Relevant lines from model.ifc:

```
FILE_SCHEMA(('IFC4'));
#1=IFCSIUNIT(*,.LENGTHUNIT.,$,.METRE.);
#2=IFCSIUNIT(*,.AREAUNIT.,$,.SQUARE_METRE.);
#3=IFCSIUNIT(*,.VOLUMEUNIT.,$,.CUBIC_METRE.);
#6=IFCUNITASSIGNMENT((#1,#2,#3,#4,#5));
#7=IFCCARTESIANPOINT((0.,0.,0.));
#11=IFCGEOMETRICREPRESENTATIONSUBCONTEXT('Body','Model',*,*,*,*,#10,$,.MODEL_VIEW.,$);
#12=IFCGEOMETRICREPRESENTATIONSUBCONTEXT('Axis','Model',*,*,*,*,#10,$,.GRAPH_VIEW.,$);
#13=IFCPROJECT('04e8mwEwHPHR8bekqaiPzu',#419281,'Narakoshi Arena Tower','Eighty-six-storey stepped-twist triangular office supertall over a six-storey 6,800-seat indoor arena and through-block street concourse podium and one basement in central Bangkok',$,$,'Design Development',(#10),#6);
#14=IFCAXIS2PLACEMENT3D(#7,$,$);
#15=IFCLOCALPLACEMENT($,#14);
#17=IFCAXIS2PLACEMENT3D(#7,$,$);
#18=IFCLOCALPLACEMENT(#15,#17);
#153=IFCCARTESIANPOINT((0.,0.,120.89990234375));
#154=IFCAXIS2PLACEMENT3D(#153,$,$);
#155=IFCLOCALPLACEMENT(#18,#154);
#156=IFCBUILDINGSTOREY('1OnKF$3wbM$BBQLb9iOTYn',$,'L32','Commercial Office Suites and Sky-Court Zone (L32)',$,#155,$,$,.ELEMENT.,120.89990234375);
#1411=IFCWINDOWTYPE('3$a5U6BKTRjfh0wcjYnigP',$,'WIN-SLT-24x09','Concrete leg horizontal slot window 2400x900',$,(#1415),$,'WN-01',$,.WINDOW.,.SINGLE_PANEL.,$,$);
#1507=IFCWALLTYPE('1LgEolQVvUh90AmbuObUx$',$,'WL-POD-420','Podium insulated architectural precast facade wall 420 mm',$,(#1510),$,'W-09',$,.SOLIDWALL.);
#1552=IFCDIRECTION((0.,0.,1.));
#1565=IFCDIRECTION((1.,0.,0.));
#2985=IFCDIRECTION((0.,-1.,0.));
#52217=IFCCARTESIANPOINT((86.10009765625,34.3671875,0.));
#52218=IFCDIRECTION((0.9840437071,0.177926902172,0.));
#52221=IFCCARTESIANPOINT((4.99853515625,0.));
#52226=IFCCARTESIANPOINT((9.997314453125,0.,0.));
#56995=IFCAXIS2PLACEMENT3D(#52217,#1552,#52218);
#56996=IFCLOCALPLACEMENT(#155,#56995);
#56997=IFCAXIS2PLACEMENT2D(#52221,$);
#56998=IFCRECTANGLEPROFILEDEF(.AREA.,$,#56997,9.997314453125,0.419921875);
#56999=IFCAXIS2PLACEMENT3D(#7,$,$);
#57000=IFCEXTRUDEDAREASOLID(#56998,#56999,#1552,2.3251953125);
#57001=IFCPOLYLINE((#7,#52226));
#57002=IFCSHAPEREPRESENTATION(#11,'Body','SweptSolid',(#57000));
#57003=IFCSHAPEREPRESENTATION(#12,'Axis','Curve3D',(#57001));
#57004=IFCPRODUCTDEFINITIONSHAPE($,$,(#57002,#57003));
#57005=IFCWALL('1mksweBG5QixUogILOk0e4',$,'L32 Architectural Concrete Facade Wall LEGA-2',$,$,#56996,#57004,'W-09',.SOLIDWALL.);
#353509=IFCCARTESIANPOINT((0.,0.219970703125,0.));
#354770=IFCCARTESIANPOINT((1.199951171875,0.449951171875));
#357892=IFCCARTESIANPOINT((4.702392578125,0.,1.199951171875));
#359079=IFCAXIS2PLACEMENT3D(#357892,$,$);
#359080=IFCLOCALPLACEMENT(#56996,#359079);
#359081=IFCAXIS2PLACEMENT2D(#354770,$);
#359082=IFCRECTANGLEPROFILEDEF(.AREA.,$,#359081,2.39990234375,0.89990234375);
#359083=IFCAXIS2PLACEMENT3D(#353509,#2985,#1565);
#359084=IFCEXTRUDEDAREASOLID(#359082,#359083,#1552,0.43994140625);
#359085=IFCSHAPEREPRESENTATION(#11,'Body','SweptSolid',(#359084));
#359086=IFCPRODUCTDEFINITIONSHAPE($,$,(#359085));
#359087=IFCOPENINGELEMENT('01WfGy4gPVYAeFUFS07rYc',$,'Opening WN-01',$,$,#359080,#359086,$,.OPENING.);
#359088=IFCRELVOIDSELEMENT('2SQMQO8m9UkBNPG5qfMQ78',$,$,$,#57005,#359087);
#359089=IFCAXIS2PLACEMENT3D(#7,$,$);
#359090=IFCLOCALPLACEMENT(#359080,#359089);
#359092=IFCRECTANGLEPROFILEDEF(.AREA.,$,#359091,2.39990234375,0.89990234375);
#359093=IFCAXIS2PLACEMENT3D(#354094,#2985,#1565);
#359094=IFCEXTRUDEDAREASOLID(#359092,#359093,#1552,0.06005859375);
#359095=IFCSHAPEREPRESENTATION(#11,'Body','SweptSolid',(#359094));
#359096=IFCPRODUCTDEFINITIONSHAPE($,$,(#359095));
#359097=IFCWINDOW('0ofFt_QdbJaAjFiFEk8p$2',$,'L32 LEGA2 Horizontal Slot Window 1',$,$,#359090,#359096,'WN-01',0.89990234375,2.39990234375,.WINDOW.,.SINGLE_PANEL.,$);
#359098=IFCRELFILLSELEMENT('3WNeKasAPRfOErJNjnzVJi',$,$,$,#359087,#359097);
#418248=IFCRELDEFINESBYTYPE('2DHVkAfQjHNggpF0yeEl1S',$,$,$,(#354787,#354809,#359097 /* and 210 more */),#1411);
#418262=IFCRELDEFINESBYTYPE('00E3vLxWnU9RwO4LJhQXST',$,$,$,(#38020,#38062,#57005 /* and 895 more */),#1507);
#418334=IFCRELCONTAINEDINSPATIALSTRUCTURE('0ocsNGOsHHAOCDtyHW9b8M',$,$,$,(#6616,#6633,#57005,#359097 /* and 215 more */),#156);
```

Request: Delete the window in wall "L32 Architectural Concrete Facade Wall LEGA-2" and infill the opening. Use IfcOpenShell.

```python
import ifcopenshell
import ifcopenshell.api.feature
import ifcopenshell.api.root
import ifcopenshell.geom
import ifcopenshell.util.shape

model = ifcopenshell.open("model.ifc")
settings = ifcopenshell.geom.settings()


def volume(element):
    """Net volume in cubic metres, openings subtracted."""
    shape = ifcopenshell.geom.create_shape(settings, element)
    return ifcopenshell.util.shape.get_volume(shape.geometry)


window = model.by_guid("0ofFt_QdbJaAjFiFEk8p$2")
opening = window.FillsVoids[0].RelatingOpeningElement
wall = opening.VoidsElements[0].RelatingBuildingElement
before = volume(wall)

ifcopenshell.api.root.remove_product(model, product=window)
ifcopenshell.api.feature.remove_feature(model, feature=opening)

after = volume(wall)

print(f"wall volume {before:.3f} -> {after:.3f} m3")

model.write("model_rev.ifc")
```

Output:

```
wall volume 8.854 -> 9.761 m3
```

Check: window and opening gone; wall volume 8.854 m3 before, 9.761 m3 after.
